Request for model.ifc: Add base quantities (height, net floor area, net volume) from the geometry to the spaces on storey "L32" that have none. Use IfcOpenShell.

First a look at what the model holds.

```python
import ifcopenshell
import ifcopenshell.util.element
import ifcopenshell.util.unit

model = ifcopenshell.open("model.ifc")
print(model.schema)
for unit_type in ("LENGTHUNIT", "AREAUNIT", "VOLUMEUNIT"):
    print(unit_type, ifcopenshell.util.unit.calculate_unit_scale(model, unit_type))
storey = next(s for s in model.by_type("IfcBuildingStorey") if s.Name == "L32")
spaces = [e for e in ifcopenshell.util.element.get_decomposition(storey) if e.is_a("IfcSpace")]
for e in sorted(spaces, key=lambda e: e.id()):
    print(e.id(), e.is_a(), e.Name, list(ifcopenshell.util.element.get_psets(e, qtos_only=True)), sep=" | ")
```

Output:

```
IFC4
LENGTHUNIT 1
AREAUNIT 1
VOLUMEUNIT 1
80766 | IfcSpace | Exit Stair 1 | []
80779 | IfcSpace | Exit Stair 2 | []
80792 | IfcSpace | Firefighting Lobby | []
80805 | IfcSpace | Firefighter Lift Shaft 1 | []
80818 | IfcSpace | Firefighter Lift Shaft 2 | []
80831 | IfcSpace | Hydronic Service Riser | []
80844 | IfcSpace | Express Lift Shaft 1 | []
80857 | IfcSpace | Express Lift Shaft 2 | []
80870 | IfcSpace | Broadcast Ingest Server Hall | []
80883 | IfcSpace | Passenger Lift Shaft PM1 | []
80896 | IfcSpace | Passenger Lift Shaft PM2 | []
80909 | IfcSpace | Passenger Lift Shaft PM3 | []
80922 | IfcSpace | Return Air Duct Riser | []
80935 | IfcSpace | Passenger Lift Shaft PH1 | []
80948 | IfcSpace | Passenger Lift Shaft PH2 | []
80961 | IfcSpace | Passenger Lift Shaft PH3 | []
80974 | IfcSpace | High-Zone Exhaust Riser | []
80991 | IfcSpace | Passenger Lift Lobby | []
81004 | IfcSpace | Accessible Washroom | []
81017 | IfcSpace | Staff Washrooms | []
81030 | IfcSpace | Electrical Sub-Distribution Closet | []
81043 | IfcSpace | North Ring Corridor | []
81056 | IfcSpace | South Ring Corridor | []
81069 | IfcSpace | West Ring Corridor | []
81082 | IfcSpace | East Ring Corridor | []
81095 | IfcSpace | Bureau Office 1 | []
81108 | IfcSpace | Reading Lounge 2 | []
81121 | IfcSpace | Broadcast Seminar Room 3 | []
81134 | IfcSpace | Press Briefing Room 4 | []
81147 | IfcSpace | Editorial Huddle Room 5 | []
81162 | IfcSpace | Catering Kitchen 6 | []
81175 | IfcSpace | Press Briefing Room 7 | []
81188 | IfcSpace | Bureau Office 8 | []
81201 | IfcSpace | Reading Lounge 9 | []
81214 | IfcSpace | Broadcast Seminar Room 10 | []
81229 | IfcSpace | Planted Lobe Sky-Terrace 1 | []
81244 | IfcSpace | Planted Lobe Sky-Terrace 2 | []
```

```python
import ifcopenshell
import ifcopenshell.api.pset
import ifcopenshell.geom
import ifcopenshell.util.element
import ifcopenshell.util.shape
import ifcopenshell.util.unit

model = ifcopenshell.open("model.ifc")
unit_scale = ifcopenshell.util.unit.calculate_unit_scale(model)
area_scale = ifcopenshell.util.unit.calculate_unit_scale(model, "AREAUNIT")
volume_scale = ifcopenshell.util.unit.calculate_unit_scale(model, "VOLUMEUNIT")
settings = ifcopenshell.geom.settings()

storey = next(s for s in model.by_type("IfcBuildingStorey") if s.Name == "L32")
spaces = [e for e in ifcopenshell.util.element.get_decomposition(storey) if e.is_a("IfcSpace")]

for e in sorted(spaces, key=lambda e: e.id()):
    if ifcopenshell.util.element.get_psets(e, qtos_only=True, should_inherit=False):
        continue
    # Geometry comes back in metres, in the element's own axes.
    shape = ifcopenshell.geom.create_shape(settings, e)
    values = {
        "Height": ifcopenshell.util.shape.get_z(shape.geometry) / unit_scale,
        "NetFloorArea": ifcopenshell.util.shape.get_footprint_area(shape.geometry) / area_scale,
        "NetVolume": ifcopenshell.util.shape.get_volume(shape.geometry) / volume_scale,
    }
    qto = ifcopenshell.api.pset.add_qto(model, product=e, name="Qto_SpaceBaseQuantities")
    ifcopenshell.api.pset.edit_qto(model, qto=qto, properties=values)
    print(e.id(), {k: round(v, 3) for k, v in values.items()})

model.write("model_edited.ifc")
```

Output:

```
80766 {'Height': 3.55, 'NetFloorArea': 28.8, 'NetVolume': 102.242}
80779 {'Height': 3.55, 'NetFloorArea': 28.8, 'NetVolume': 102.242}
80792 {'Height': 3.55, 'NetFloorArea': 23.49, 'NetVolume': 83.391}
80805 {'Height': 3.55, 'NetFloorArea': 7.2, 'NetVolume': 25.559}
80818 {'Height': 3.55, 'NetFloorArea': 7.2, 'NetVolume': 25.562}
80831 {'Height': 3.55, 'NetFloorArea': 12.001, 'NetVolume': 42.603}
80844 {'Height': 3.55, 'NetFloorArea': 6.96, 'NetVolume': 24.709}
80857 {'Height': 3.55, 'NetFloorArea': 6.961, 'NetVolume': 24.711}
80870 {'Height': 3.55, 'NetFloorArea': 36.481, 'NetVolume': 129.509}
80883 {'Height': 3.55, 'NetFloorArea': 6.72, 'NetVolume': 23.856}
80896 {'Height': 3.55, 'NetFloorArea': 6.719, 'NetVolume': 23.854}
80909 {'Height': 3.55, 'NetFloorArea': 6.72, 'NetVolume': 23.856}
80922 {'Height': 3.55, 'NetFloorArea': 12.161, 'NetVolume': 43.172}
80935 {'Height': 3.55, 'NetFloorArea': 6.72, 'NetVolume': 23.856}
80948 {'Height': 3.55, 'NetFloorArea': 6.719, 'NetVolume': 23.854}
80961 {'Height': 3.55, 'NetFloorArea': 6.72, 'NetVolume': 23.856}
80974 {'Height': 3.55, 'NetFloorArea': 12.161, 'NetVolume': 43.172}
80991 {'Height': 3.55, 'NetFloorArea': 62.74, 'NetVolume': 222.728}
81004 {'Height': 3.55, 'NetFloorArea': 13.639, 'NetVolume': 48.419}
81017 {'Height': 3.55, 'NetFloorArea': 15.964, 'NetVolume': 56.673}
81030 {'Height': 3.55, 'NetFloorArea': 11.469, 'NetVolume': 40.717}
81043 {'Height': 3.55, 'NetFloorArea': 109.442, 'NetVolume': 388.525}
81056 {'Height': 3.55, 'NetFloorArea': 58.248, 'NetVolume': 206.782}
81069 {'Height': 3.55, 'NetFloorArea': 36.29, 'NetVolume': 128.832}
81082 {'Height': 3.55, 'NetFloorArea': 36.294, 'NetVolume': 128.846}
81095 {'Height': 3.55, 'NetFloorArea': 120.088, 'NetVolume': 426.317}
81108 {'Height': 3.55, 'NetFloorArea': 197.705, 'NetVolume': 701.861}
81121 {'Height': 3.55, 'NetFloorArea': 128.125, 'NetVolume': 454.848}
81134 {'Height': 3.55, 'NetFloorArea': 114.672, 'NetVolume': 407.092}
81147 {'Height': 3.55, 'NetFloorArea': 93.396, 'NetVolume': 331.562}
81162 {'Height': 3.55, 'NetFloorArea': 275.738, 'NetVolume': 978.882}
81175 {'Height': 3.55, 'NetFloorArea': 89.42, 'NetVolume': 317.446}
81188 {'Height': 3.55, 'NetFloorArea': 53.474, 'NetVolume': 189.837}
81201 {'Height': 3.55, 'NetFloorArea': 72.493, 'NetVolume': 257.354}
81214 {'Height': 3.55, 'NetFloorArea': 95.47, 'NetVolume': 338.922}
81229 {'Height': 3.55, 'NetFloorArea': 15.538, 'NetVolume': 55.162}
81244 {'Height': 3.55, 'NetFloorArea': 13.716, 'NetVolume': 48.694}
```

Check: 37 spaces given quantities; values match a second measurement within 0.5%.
